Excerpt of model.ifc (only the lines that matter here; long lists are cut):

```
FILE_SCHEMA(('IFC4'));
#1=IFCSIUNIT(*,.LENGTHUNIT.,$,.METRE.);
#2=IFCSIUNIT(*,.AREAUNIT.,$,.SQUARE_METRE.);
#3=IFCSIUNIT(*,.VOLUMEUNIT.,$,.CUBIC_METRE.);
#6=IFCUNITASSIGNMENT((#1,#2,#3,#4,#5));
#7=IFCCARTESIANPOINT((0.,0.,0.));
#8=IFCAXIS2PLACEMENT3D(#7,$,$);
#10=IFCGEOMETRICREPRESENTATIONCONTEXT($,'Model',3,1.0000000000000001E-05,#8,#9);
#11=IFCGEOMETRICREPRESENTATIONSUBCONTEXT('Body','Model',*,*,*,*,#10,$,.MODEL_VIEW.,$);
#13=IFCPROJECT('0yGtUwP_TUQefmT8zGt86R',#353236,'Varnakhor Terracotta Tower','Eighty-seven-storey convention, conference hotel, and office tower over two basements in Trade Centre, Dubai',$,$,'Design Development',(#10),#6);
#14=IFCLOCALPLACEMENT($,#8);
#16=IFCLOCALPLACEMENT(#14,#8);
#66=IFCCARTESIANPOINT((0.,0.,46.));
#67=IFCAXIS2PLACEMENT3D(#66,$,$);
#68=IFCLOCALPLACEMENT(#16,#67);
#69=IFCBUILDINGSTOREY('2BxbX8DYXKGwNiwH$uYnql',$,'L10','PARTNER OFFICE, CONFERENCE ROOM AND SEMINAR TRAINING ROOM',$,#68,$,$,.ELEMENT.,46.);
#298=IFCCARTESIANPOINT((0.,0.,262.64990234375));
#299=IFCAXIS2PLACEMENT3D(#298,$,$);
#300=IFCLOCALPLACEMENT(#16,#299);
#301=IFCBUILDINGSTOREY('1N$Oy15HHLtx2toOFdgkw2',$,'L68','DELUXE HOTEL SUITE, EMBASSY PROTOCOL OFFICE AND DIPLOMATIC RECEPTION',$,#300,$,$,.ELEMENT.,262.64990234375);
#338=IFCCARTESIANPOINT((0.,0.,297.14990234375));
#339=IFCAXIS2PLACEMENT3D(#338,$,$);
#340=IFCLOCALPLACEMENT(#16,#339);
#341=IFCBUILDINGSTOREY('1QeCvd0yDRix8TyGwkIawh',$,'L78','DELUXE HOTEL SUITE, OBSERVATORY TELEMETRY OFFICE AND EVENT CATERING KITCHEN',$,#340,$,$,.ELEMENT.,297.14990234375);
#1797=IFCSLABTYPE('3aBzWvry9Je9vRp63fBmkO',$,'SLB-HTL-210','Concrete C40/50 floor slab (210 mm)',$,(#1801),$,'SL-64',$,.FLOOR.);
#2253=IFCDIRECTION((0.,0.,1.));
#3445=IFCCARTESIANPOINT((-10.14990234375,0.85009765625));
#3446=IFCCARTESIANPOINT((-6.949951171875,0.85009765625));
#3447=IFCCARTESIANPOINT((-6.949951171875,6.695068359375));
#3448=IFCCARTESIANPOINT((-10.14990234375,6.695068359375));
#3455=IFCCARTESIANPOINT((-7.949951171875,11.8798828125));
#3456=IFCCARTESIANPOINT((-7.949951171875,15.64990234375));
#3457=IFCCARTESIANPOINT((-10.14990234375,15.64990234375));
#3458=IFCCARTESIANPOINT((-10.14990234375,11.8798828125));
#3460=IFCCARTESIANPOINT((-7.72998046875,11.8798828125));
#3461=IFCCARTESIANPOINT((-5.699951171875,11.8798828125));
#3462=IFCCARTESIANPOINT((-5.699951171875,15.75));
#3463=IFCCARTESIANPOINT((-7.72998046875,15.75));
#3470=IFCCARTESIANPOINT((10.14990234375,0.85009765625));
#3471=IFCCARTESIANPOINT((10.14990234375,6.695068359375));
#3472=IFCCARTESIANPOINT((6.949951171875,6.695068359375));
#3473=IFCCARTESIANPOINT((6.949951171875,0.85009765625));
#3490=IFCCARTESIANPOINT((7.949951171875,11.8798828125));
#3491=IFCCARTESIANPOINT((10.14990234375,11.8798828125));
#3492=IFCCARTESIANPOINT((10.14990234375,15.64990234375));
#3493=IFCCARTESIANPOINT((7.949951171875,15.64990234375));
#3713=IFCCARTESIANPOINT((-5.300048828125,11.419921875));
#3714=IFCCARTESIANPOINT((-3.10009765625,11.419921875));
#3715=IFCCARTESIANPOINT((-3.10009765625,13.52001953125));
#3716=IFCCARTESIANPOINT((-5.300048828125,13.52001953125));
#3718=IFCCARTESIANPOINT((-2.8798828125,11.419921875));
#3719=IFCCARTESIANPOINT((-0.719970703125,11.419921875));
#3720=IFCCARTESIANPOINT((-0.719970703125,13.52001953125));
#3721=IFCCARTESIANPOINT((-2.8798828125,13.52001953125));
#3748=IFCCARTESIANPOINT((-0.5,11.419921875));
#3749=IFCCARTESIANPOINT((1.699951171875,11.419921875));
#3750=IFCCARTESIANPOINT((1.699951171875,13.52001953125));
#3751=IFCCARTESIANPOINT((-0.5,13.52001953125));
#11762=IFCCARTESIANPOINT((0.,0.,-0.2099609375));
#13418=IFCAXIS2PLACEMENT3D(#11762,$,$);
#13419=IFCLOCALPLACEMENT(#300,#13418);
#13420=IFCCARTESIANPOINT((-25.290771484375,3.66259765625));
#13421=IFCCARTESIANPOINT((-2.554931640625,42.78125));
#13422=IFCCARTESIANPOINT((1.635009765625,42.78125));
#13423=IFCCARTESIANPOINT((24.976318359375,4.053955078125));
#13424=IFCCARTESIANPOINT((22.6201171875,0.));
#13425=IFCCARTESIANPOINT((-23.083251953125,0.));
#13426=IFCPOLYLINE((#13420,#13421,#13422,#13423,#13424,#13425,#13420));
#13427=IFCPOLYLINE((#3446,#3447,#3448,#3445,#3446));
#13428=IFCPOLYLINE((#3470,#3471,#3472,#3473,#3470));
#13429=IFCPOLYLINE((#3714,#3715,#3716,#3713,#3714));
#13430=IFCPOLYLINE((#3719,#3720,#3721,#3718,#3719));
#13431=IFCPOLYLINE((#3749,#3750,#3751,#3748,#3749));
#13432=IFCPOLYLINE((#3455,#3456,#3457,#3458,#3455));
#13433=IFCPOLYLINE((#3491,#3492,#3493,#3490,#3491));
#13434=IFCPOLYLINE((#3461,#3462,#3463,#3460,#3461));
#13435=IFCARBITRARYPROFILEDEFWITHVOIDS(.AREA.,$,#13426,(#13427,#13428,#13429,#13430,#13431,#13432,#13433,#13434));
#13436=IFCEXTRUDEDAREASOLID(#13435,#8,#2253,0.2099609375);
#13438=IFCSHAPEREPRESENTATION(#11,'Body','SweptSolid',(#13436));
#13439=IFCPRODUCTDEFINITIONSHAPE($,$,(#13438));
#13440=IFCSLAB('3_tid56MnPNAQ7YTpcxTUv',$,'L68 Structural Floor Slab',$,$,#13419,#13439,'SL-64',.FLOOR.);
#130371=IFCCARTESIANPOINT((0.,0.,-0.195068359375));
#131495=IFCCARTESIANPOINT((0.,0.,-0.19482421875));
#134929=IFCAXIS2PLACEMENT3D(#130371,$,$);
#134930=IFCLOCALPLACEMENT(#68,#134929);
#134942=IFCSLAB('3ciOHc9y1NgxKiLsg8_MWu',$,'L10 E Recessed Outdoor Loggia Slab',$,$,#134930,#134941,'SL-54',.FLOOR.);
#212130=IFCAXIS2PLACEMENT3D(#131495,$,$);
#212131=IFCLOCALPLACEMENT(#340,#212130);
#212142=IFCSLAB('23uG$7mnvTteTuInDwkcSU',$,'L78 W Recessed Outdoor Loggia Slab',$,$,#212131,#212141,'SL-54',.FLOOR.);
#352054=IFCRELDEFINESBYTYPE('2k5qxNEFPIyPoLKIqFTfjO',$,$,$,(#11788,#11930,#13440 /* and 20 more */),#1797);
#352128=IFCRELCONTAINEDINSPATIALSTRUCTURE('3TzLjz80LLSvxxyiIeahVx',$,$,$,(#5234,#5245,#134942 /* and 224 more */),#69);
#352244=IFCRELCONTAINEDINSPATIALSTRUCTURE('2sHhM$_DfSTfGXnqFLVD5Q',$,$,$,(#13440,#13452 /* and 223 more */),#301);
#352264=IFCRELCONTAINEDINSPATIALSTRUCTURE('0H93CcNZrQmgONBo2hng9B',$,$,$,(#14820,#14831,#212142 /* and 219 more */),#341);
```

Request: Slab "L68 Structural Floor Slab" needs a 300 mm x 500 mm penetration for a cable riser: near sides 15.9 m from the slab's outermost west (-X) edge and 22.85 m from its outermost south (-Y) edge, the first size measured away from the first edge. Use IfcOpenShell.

```python
import numpy as np
import ifcopenshell
import ifcopenshell.api.feature
import ifcopenshell.api.geometry
import ifcopenshell.api.root
import ifcopenshell.geom
import ifcopenshell.util.placement
import ifcopenshell.util.representation
import ifcopenshell.util.shape
import ifcopenshell.util.unit

model = ifcopenshell.open("model.ifc")
unit_scale = ifcopenshell.util.unit.calculate_unit_scale(model)
settings = ifcopenshell.geom.settings()


def volume(element):
    """Net volume in cubic metres, openings subtracted."""
    shape = ifcopenshell.geom.create_shape(settings, element)
    return ifcopenshell.util.shape.get_volume(shape.geometry)


slab = model.by_id(13440)
before = volume(slab)

# Extent in the slab's own axes, in metres. The edges named are its -X and -Y sides.
slab_shape = ifcopenshell.geom.create_shape(settings, slab)
vertices = ifcopenshell.util.shape.get_vertices(slab_shape.geometry)
x_min, y_min, bottom = vertices.min(axis=0)
top = vertices[:, 2].max()

opening = ifcopenshell.api.root.create_entity(model, ifc_class="IfcOpeningElement", name="Cable riser opening", predefined_type="OPENING")
context = ifcopenshell.util.representation.get_context(model, "Model", "Body", "MODEL_VIEW")
width, depth = 0.3, 0.5
outline = [(0.0, 0.0), (width, 0.0), (width, depth), (0.0, depth), (0.0, 0.0)]
# Overshoot both faces by 50 mm so the cut is clean.
shape = ifcopenshell.api.geometry.add_slab_representation(
    model, context=context, depth=top - bottom + 0.1, polyline=outline
)
ifcopenshell.api.geometry.assign_representation(model, product=opening, representation=shape)

matrix = ifcopenshell.util.placement.get_local_placement(slab.ObjectPlacement)
matrix[:, 3] = matrix @ np.append(np.array([x_min + 15.9, y_min + 22.85, bottom - 0.05]) / unit_scale, 1.0)
ifcopenshell.api.geometry.edit_object_placement(model, product=opening, matrix=matrix, is_si=False)
ifcopenshell.api.feature.add_feature(model, feature=opening, element=slab)

after = volume(slab)

print(f"slab volume {before:.3f} -> {after:.3f} m3")

model.write("model-out.ifc")
```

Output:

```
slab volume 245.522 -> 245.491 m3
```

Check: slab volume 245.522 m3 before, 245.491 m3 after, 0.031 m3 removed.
